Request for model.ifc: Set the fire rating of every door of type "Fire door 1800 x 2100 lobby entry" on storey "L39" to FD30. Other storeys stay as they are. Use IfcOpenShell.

First a look at what the model holds.

```python
import ifcopenshell
import ifcopenshell.util.element

model = ifcopenshell.open("model.ifc")
print(model.schema)
storey = next(s for s in model.by_type("IfcBuildingStorey") if s.Name == "L39")
doors = [e for e in ifcopenshell.util.element.get_decomposition(storey) if e.is_a("IfcDoor")]
seen = {}
for e in doors:
    element_type = ifcopenshell.util.element.get_type(e)
    key = (element_type.Name if element_type != e and element_type else None, ifcopenshell.util.element.get_pset(e, "Pset_DoorCommon", "FireRating"))
    seen[key] = seen.get(key, 0) + 1
for (name, value), count in sorted(seen.items(), key=str):
    print(count, "x", name, "|", value)
```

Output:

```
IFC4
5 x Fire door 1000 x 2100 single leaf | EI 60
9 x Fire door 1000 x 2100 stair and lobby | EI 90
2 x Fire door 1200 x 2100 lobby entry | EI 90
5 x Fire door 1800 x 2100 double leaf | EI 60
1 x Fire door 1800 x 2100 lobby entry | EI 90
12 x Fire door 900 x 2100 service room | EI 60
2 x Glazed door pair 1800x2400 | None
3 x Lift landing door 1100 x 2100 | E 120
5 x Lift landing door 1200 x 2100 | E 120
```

```python
import ifcopenshell
import ifcopenshell.api.pset
import ifcopenshell.util.element

model = ifcopenshell.open("model.ifc")

storey = next(s for s in model.by_type("IfcBuildingStorey") if s.Name == "L39")
doors = [e for e in ifcopenshell.util.element.get_decomposition(storey) if e.is_a("IfcDoor")]

count = 0
for e in doors:
    element_type = ifcopenshell.util.element.get_type(e)
    if element_type in (None, e) or element_type.Name != "Fire door 1800 x 2100 lobby entry":
        continue
    found = ifcopenshell.util.element.get_pset(e, "Pset_DoorCommon", should_inherit=False)
    if found:
        pset = model.by_id(found["id"])
        if len(ifcopenshell.util.element.get_elements_by_pset(pset)) > 1:
            pset = ifcopenshell.api.pset.unshare_pset(model, products=[e], pset=pset)[0]
    else:
        pset = ifcopenshell.api.pset.add_pset(model, product=e, name="Pset_DoorCommon")
    ifcopenshell.api.pset.edit_pset(model, pset=pset, properties={"FireRating": "FD30"})
    count += 1

print(count, "doors updated")

model.write("model_v2.ifc")
```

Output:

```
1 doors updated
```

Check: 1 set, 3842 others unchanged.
